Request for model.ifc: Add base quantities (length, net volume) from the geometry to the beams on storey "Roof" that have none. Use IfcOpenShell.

First a look at what the model holds.

```python
import ifcopenshell
import ifcopenshell.util.element
import ifcopenshell.util.unit

model = ifcopenshell.open("model.ifc")
print(model.schema)
for unit_type in ("LENGTHUNIT", "AREAUNIT", "VOLUMEUNIT"):
    print(unit_type, ifcopenshell.util.unit.calculate_unit_scale(model, unit_type))
storey = next(s for s in model.by_type("IfcBuildingStorey") if s.Name == "Roof")
beams = [e for e in ifcopenshell.util.element.get_decomposition(storey) if e.is_a("IfcBeam")]
for e in sorted(beams, key=lambda e: e.id()):
    print(e.id(), e.is_a(), e.Name, list(ifcopenshell.util.element.get_psets(e, qtos_only=True)), sep=" | ")
```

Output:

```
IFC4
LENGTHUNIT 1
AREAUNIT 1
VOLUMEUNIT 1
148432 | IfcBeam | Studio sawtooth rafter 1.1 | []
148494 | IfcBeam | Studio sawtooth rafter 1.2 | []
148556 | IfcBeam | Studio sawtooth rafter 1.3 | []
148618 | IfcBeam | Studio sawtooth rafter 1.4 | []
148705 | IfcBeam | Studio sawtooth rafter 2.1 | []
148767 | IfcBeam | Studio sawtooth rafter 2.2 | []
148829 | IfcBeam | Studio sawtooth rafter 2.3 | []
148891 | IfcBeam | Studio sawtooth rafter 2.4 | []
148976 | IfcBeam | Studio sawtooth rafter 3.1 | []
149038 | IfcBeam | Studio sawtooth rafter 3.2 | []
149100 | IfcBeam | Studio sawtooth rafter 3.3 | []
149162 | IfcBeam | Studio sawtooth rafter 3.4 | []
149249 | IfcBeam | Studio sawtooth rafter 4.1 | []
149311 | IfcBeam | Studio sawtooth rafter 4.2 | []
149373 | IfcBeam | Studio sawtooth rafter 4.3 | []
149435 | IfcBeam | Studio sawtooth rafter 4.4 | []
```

```python
import ifcopenshell
import ifcopenshell.api.pset
import ifcopenshell.geom
import ifcopenshell.util.element
import ifcopenshell.util.shape
import ifcopenshell.util.unit

model = ifcopenshell.open("model.ifc")
unit_scale = ifcopenshell.util.unit.calculate_unit_scale(model)
volume_scale = ifcopenshell.util.unit.calculate_unit_scale(model, "VOLUMEUNIT")
settings = ifcopenshell.geom.settings()

storey = next(s for s in model.by_type("IfcBuildingStorey") if s.Name == "Roof")
beams = [e for e in ifcopenshell.util.element.get_decomposition(storey) if e.is_a("IfcBeam")]

for e in sorted(beams, key=lambda e: e.id()):
    if ifcopenshell.util.element.get_psets(e, qtos_only=True, should_inherit=False):
        continue
    # Geometry comes back in metres, in the element's own axes.
    shape = ifcopenshell.geom.create_shape(settings, e)
    values = {
        "Length": ifcopenshell.util.shape.get_max_xyz(shape.geometry) / unit_scale,
        "NetVolume": ifcopenshell.util.shape.get_volume(shape.geometry) / volume_scale,
    }
    qto = ifcopenshell.api.pset.add_qto(model, product=e, name="Qto_BeamBaseQuantities")
    ifcopenshell.api.pset.edit_qto(model, qto=qto, properties=values)
    print(e.id(), {k: round(v, 3) for k, v in values.items()})

model.write("model_edited.ifc")
```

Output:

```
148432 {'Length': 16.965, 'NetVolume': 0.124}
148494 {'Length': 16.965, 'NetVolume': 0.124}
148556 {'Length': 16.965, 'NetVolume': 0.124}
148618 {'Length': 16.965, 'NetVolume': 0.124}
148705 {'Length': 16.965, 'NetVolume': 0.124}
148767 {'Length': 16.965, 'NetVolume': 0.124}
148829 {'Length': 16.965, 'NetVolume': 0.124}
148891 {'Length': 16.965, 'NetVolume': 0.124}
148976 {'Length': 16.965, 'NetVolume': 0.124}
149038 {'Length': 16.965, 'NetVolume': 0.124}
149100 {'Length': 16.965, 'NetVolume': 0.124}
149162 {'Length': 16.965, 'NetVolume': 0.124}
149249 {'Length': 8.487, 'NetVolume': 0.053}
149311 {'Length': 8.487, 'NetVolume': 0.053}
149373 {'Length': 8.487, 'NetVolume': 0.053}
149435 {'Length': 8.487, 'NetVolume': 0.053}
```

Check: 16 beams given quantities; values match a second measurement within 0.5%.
